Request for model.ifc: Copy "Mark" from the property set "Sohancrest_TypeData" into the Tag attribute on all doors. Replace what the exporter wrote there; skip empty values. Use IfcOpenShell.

First a look at what the model holds.

```python
import ifcopenshell
import ifcopenshell.util.element

model = ifcopenshell.open("model.ifc")
print(model.schema)
doors = model.by_type("IfcDoor")
print(len(doors), "doors")
for e in doors[:8]:
    source = ifcopenshell.util.element.get_pset(e, "Sohancrest_TypeData", "Mark")
    target = e.Tag
    print(e.id(), repr(source), repr(target), sep=" | ")
```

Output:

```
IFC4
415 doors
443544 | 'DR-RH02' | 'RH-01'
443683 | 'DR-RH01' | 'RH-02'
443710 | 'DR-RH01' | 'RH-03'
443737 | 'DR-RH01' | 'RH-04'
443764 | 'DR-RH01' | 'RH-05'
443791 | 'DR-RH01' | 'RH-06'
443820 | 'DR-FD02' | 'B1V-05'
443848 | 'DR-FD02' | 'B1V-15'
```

```python
import ifcopenshell
import ifcopenshell.util.element

model = ifcopenshell.open("model.ifc")

count = 0
for e in model.by_type("IfcDoor"):
    value = ifcopenshell.util.element.get_pset(e, "Sohancrest_TypeData", "Mark")
    current = e.Tag
    if not value or not value.strip() or current == value:
        continue
    e.Tag = value
    count += 1

print(count, "doors updated")

model.write("model-out.ifc")
```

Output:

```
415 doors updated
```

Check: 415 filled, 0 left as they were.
